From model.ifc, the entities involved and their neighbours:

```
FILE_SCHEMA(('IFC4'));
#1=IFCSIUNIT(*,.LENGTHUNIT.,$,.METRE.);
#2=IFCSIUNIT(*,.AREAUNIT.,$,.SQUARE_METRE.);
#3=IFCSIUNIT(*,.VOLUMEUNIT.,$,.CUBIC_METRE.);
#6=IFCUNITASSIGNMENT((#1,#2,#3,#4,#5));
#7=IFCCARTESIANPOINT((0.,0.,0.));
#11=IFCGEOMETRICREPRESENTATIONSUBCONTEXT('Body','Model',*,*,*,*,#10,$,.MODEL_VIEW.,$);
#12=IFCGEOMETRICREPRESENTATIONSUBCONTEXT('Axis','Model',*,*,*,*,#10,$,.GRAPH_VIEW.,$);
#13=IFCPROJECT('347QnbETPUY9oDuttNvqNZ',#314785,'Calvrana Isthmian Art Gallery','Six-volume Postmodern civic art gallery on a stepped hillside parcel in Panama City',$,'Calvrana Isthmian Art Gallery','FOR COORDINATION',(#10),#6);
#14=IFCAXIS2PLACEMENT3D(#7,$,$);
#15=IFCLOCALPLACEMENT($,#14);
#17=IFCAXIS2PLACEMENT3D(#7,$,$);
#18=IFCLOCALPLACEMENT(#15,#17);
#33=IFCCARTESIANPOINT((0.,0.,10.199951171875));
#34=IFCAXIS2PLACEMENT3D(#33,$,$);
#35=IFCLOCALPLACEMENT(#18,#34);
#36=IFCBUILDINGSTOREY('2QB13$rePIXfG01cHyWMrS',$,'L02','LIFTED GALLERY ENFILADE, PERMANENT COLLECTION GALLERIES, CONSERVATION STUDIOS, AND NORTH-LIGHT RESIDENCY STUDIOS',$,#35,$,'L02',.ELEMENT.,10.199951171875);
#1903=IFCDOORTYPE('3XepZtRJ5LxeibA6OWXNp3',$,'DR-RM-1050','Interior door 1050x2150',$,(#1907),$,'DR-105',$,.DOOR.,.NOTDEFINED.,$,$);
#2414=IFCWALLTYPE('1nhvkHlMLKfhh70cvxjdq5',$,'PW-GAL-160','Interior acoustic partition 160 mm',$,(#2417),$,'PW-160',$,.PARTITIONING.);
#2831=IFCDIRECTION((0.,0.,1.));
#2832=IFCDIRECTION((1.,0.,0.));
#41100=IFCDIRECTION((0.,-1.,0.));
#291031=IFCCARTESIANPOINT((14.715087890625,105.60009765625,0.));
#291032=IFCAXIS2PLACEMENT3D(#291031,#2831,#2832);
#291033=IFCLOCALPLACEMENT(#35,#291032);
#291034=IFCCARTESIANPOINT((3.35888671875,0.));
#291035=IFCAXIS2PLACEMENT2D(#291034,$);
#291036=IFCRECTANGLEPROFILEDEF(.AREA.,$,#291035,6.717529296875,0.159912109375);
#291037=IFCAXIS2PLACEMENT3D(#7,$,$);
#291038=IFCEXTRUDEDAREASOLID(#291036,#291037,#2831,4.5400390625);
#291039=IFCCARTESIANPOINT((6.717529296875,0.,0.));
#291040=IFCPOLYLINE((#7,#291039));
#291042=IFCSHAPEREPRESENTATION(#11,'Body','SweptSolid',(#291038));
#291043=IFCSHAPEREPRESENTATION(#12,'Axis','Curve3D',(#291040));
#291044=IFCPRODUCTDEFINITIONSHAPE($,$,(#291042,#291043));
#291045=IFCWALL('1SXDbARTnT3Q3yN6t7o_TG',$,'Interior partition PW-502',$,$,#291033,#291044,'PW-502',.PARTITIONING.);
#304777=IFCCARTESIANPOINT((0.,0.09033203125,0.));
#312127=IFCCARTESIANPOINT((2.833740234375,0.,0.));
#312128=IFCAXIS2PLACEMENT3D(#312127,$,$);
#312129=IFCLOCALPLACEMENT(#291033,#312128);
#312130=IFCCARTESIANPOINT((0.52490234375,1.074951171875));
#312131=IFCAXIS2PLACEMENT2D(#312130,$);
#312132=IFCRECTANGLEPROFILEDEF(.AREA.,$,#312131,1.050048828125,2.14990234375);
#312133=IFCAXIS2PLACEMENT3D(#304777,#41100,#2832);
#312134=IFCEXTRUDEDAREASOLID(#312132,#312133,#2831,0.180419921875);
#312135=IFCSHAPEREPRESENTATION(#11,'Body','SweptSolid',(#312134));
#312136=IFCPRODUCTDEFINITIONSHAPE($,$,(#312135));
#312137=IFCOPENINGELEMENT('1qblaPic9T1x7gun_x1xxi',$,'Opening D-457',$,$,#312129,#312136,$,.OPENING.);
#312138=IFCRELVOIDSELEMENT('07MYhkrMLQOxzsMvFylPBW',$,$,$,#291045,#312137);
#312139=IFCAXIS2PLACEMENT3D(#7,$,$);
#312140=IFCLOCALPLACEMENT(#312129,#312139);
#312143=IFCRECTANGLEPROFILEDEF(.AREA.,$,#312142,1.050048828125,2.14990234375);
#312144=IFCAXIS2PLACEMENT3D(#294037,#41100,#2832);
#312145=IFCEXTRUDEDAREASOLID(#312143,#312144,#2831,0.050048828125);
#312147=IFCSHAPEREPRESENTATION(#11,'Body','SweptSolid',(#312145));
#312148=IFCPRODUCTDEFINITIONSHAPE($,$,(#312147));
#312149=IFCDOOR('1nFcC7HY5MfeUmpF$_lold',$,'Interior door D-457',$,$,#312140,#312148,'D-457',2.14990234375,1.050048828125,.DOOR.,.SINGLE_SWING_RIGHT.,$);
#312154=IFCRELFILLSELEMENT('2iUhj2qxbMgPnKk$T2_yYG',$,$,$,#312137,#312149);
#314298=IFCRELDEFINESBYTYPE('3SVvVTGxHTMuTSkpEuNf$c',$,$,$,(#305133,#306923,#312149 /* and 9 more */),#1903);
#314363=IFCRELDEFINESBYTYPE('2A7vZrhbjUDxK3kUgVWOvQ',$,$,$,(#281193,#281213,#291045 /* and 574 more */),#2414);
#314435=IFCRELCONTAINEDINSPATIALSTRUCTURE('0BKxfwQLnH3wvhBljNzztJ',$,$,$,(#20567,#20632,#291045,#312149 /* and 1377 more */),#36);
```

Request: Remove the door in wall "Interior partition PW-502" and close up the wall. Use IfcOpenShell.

```python
import ifcopenshell
import ifcopenshell.api.feature
import ifcopenshell.api.root
import ifcopenshell.geom
import ifcopenshell.util.shape

model = ifcopenshell.open("model.ifc")
settings = ifcopenshell.geom.settings()


def volume(element):
    """Net volume in cubic metres, openings subtracted."""
    shape = ifcopenshell.geom.create_shape(settings, element)
    return ifcopenshell.util.shape.get_volume(shape.geometry)


door = model.by_guid("1nFcC7HY5MfeUmpF$_lold")
opening = door.FillsVoids[0].RelatingOpeningElement
wall = opening.VoidsElements[0].RelatingBuildingElement
before = volume(wall)

ifcopenshell.api.root.remove_product(model, product=door)
ifcopenshell.api.feature.remove_feature(model, feature=opening)

after = volume(wall)

print(f"wall volume {before:.3f} -> {after:.3f} m3")

model.write("model_updated.ifc")
```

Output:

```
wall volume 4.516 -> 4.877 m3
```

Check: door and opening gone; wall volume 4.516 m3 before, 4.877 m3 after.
